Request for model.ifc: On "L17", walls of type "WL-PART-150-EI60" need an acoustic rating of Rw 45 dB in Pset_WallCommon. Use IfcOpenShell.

First a look at what the model holds.

```python
import ifcopenshell
import ifcopenshell.util.element

model = ifcopenshell.open("model.ifc")
print(model.schema)
storey = next(s for s in model.by_type("IfcBuildingStorey") if s.Name == "L17")
walls = [e for e in ifcopenshell.util.element.get_decomposition(storey) if e.is_a("IfcWall")]
seen = {}
for e in walls:
    element_type = ifcopenshell.util.element.get_type(e)
    key = (element_type.Name if element_type != e and element_type else None, ifcopenshell.util.element.get_pset(e, "Pset_WallCommon", "AcousticRating"))
    seen[key] = seen.get(key, 0) + 1
for (name, value), count in sorted(seen.items(), key=str):
    print(count, "x", name, "|", value)
```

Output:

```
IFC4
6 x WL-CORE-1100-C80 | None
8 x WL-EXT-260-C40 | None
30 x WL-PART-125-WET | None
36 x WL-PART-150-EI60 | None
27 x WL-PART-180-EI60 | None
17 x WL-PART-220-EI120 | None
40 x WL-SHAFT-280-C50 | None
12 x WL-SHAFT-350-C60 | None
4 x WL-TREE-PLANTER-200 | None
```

```python
import ifcopenshell
import ifcopenshell.api.pset
import ifcopenshell.util.element

model = ifcopenshell.open("model.ifc")

storey = next(s for s in model.by_type("IfcBuildingStorey") if s.Name == "L17")
walls = [e for e in ifcopenshell.util.element.get_decomposition(storey) if e.is_a("IfcWall")]

count = 0
for e in walls:
    element_type = ifcopenshell.util.element.get_type(e)
    if element_type in (None, e) or element_type.Name != "WL-PART-150-EI60":
        continue
    # add_pset returns the element's existing set when there is one.
    pset = ifcopenshell.api.pset.add_pset(model, product=e, name="Pset_WallCommon")
    ifcopenshell.api.pset.edit_pset(model, pset=pset, properties={"AcousticRating": "Rw 45 dB"})
    count += 1

print(count, "walls updated")

model.write("model_updated.ifc")
```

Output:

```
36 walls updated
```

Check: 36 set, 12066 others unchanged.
